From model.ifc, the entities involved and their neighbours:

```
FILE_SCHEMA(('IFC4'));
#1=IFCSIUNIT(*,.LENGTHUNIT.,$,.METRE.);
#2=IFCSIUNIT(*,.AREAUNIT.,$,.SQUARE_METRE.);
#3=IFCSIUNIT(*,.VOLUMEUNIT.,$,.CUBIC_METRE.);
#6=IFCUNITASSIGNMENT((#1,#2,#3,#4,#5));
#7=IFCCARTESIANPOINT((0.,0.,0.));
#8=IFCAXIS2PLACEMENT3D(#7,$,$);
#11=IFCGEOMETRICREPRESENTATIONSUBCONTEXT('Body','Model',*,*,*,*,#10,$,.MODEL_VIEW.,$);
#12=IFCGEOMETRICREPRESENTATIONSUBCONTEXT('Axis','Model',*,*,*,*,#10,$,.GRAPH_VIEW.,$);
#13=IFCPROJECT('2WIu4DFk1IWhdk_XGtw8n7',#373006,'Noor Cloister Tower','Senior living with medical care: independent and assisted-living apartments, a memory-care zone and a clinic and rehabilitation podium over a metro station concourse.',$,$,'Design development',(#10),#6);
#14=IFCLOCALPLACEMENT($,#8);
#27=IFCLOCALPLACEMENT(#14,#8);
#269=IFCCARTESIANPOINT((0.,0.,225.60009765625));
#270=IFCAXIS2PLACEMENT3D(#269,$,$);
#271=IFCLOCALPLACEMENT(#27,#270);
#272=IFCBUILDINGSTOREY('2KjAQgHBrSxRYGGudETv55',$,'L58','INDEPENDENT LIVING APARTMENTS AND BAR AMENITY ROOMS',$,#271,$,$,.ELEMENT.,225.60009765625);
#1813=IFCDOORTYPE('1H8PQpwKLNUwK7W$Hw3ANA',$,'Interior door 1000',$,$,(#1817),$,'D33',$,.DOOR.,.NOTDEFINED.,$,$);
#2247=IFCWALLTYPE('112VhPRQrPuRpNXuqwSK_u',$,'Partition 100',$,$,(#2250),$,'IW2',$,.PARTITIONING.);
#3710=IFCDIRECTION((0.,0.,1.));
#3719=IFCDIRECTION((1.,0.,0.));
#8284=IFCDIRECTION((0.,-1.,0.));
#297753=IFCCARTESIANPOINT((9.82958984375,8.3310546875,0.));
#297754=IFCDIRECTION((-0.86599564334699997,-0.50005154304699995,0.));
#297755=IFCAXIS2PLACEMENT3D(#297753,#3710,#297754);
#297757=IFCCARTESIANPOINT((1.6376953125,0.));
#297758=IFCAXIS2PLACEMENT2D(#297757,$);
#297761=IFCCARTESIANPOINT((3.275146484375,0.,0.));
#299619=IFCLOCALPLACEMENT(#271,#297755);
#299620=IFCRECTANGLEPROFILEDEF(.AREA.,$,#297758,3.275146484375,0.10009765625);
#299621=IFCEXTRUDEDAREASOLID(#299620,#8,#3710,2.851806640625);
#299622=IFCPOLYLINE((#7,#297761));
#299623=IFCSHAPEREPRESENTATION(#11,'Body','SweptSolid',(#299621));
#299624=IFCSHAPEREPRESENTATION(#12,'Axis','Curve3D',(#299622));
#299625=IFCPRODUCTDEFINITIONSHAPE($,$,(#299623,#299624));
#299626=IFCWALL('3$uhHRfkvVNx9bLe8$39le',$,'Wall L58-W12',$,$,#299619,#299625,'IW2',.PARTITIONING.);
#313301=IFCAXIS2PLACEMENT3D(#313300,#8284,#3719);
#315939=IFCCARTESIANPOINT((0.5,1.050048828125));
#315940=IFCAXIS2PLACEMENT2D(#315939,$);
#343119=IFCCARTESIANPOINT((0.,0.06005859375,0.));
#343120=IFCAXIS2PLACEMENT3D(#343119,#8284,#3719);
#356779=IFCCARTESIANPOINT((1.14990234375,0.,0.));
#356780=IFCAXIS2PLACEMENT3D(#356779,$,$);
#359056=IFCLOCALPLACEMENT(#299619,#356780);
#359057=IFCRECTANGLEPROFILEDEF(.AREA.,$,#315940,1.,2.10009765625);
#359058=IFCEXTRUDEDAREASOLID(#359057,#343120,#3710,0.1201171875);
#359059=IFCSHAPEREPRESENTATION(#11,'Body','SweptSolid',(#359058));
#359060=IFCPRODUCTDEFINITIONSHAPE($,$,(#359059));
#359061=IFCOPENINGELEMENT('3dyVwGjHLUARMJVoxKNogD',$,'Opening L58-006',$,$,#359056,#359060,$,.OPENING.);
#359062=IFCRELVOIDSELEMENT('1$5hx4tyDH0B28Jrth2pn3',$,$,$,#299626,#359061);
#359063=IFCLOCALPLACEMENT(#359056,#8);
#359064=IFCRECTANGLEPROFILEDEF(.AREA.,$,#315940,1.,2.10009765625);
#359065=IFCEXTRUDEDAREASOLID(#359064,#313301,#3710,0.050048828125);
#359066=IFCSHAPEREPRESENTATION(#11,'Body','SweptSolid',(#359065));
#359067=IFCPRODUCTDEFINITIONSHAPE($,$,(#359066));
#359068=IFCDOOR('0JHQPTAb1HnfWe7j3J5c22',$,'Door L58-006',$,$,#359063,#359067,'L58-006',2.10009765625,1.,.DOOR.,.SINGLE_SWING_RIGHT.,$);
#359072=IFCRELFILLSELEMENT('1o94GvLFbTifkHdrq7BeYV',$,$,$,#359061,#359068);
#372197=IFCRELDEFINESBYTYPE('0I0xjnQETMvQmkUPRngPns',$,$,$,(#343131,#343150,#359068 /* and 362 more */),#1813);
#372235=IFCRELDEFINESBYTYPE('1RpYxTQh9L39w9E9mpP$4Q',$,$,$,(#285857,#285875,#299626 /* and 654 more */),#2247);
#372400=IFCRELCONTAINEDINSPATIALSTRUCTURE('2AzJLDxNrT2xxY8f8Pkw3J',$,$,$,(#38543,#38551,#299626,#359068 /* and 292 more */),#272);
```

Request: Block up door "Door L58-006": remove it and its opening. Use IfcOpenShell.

```python
import ifcopenshell
import ifcopenshell.api.feature
import ifcopenshell.api.root
import ifcopenshell.geom
import ifcopenshell.util.shape

model = ifcopenshell.open("model.ifc")
settings = ifcopenshell.geom.settings()


def volume(element):
    """Net volume in cubic metres, openings subtracted."""
    shape = ifcopenshell.geom.create_shape(settings, element)
    return ifcopenshell.util.shape.get_volume(shape.geometry)


door = model.by_guid("0JHQPTAb1HnfWe7j3J5c22")
opening = door.FillsVoids[0].RelatingOpeningElement
wall = opening.VoidsElements[0].RelatingBuildingElement
before = volume(wall)

ifcopenshell.api.root.remove_product(model, product=door)
ifcopenshell.api.feature.remove_feature(model, feature=opening)

after = volume(wall)

print(f"wall volume {before:.3f} -> {after:.3f} m3")

model.write("model_edited.ifc")
```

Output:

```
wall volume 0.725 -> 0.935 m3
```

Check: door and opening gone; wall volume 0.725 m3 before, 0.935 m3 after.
